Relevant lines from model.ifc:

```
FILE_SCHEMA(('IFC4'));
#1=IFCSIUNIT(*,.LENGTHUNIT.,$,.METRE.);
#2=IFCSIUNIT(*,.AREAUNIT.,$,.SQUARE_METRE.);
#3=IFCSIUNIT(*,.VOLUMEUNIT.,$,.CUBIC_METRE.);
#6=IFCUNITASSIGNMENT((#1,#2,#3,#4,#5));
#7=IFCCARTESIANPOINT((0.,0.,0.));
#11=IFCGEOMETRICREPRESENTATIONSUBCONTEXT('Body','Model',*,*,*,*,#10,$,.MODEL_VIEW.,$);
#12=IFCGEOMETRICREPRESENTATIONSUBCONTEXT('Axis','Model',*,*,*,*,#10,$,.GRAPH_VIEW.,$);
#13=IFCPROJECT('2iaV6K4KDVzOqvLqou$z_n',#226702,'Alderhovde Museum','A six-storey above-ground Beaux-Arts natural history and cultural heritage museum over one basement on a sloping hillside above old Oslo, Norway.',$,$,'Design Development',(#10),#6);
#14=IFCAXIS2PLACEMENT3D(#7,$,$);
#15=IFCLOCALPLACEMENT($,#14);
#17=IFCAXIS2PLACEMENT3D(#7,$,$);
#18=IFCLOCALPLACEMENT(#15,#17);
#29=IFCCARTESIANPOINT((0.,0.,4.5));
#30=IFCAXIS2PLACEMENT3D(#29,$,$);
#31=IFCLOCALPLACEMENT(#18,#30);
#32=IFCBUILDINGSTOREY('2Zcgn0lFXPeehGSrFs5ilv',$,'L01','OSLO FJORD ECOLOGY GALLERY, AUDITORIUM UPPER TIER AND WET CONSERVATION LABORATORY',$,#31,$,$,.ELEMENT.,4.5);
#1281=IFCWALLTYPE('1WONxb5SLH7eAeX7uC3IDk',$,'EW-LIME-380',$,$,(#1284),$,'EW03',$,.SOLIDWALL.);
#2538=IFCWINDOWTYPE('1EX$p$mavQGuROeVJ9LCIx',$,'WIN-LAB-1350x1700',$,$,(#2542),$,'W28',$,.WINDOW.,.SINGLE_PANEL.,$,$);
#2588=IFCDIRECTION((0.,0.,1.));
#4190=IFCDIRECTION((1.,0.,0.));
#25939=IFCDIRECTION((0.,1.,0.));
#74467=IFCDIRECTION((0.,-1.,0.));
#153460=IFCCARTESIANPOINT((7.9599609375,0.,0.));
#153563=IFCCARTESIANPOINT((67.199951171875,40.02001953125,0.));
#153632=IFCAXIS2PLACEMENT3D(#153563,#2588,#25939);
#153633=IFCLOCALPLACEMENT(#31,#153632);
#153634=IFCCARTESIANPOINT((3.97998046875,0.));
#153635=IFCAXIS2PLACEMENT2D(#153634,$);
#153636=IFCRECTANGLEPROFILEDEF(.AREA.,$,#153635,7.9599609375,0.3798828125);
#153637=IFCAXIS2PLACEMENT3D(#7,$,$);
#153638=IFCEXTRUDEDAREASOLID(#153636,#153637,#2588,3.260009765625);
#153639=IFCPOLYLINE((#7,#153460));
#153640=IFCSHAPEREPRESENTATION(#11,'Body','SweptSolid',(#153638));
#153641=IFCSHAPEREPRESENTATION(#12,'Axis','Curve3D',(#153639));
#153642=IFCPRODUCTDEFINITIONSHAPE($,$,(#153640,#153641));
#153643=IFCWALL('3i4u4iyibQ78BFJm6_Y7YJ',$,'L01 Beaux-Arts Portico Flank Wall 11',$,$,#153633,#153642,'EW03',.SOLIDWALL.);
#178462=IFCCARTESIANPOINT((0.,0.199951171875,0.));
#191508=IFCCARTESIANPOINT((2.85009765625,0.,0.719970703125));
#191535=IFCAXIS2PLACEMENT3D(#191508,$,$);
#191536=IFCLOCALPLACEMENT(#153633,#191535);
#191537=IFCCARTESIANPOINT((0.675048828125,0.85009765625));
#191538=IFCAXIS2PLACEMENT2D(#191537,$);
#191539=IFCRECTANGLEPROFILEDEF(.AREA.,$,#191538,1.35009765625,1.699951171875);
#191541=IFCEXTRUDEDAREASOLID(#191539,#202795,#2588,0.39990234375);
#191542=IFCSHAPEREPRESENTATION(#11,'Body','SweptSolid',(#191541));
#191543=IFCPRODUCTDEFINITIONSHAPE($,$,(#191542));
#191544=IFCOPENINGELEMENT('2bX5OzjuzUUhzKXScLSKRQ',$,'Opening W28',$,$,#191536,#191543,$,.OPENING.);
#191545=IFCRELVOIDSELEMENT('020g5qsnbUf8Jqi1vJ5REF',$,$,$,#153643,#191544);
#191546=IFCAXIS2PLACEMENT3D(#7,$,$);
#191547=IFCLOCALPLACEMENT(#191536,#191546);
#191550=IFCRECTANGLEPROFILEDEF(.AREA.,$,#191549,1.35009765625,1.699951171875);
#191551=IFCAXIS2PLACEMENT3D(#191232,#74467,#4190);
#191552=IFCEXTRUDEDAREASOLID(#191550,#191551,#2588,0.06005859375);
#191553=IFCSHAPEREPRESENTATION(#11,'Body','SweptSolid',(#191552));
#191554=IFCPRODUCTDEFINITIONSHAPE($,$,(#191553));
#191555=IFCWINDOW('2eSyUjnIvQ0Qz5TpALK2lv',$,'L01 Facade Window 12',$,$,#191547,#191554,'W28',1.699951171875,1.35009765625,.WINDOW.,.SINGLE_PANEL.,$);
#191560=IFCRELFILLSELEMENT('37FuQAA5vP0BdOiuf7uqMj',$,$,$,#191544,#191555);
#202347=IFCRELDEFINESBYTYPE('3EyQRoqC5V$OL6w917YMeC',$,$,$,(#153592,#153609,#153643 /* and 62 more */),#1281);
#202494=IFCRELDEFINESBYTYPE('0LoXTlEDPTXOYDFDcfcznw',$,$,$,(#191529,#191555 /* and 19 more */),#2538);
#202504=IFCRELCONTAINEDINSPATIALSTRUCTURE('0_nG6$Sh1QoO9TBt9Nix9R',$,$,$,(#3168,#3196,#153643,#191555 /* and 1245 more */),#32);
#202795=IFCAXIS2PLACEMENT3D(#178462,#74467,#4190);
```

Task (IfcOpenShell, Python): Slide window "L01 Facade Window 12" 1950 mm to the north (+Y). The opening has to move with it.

```python
import ifcopenshell
import ifcopenshell.api.geometry
import ifcopenshell.util.placement
import ifcopenshell.util.unit

model = ifcopenshell.open("model.ifc")
unit_scale = ifcopenshell.util.unit.calculate_unit_scale(model)

window = model.by_id(191555)
opening = window.FillsVoids[0].RelatingOpeningElement
wall = opening.VoidsElements[0].RelatingBuildingElement

wall_matrix = ifcopenshell.util.placement.get_local_placement(wall.ObjectPlacement)
shift = wall_matrix[:3, 0] * 1.95 / unit_scale
before = ifcopenshell.util.placement.get_local_placement(window.ObjectPlacement)[:3, 3].copy()

# The window is placed relative to its opening, so it follows when the opening moves.
matrix = ifcopenshell.util.placement.get_local_placement(opening.ObjectPlacement)
matrix[:3, 3] += shift
ifcopenshell.api.geometry.edit_object_placement(
    model, product=opening, matrix=matrix, is_si=False, should_transform_children=True
)

after = ifcopenshell.util.placement.get_local_placement(window.ObjectPlacement)[:3, 3]
print("window moved by", (after - before).round(3) + 0.0)

model.write("model_updated.ifc")
```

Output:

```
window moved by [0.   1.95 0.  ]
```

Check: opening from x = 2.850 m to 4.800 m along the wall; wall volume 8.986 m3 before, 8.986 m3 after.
